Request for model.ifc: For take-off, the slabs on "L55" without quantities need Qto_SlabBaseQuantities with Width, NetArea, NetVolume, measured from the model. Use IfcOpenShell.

First a look at what the model holds.

```python
import ifcopenshell
import ifcopenshell.util.element
import ifcopenshell.util.unit

model = ifcopenshell.open("model.ifc")
print(model.schema)
for unit_type in ("LENGTHUNIT", "AREAUNIT", "VOLUMEUNIT"):
    print(unit_type, ifcopenshell.util.unit.calculate_unit_scale(model, unit_type))
storey = next(s for s in model.by_type("IfcBuildingStorey") if s.Name == "L55")
slabs = [e for e in ifcopenshell.util.element.get_decomposition(storey) if e.is_a("IfcSlab")]
for e in sorted(slabs, key=lambda e: e.id()):
    print(e.id(), e.is_a(), e.Name, list(ifcopenshell.util.element.get_psets(e, qtos_only=True)), sep=" | ")
```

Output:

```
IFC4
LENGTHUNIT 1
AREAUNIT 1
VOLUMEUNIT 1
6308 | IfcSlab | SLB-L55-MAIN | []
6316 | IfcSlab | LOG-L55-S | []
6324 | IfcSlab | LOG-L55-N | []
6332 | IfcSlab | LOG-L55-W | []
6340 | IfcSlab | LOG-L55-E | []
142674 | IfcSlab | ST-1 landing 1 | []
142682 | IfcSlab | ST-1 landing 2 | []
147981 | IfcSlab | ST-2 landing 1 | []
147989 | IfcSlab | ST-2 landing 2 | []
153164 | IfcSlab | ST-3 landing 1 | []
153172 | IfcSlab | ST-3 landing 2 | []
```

```python
import ifcopenshell
import ifcopenshell.api.pset
import ifcopenshell.geom
import ifcopenshell.util.element
import ifcopenshell.util.shape
import ifcopenshell.util.unit

model = ifcopenshell.open("model.ifc")
unit_scale = ifcopenshell.util.unit.calculate_unit_scale(model)
area_scale = ifcopenshell.util.unit.calculate_unit_scale(model, "AREAUNIT")
volume_scale = ifcopenshell.util.unit.calculate_unit_scale(model, "VOLUMEUNIT")
settings = ifcopenshell.geom.settings()

storey = next(s for s in model.by_type("IfcBuildingStorey") if s.Name == "L55")
slabs = [e for e in ifcopenshell.util.element.get_decomposition(storey) if e.is_a("IfcSlab")]

for e in sorted(slabs, key=lambda e: e.id()):
    if ifcopenshell.util.element.get_psets(e, qtos_only=True, should_inherit=False):
        continue
    # Geometry comes back in metres, in the element's own axes.
    shape = ifcopenshell.geom.create_shape(settings, e)
    values = {
        "Width": ifcopenshell.util.shape.get_z(shape.geometry) / unit_scale,
        "NetArea": ifcopenshell.util.shape.get_footprint_area(shape.geometry) / area_scale,
        "NetVolume": ifcopenshell.util.shape.get_volume(shape.geometry) / volume_scale,
    }
    qto = ifcopenshell.api.pset.add_qto(model, product=e, name="Qto_SlabBaseQuantities")
    ifcopenshell.api.pset.edit_qto(model, qto=qto, properties=values)
    print(e.id(), {k: round(v, 3) for k, v in values.items()})

model.write("model_updated.ifc")
```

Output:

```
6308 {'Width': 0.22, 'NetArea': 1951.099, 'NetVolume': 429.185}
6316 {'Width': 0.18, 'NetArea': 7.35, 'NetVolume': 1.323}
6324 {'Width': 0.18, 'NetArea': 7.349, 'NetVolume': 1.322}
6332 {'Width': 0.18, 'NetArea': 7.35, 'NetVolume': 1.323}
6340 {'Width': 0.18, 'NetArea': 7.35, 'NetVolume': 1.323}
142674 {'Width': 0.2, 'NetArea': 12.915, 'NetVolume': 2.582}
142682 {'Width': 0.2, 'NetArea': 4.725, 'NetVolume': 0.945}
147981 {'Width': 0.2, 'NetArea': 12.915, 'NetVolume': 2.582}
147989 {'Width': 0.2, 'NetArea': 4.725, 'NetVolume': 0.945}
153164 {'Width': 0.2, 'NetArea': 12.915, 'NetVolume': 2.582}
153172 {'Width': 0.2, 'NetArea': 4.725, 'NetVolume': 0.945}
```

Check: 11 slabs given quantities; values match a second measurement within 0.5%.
